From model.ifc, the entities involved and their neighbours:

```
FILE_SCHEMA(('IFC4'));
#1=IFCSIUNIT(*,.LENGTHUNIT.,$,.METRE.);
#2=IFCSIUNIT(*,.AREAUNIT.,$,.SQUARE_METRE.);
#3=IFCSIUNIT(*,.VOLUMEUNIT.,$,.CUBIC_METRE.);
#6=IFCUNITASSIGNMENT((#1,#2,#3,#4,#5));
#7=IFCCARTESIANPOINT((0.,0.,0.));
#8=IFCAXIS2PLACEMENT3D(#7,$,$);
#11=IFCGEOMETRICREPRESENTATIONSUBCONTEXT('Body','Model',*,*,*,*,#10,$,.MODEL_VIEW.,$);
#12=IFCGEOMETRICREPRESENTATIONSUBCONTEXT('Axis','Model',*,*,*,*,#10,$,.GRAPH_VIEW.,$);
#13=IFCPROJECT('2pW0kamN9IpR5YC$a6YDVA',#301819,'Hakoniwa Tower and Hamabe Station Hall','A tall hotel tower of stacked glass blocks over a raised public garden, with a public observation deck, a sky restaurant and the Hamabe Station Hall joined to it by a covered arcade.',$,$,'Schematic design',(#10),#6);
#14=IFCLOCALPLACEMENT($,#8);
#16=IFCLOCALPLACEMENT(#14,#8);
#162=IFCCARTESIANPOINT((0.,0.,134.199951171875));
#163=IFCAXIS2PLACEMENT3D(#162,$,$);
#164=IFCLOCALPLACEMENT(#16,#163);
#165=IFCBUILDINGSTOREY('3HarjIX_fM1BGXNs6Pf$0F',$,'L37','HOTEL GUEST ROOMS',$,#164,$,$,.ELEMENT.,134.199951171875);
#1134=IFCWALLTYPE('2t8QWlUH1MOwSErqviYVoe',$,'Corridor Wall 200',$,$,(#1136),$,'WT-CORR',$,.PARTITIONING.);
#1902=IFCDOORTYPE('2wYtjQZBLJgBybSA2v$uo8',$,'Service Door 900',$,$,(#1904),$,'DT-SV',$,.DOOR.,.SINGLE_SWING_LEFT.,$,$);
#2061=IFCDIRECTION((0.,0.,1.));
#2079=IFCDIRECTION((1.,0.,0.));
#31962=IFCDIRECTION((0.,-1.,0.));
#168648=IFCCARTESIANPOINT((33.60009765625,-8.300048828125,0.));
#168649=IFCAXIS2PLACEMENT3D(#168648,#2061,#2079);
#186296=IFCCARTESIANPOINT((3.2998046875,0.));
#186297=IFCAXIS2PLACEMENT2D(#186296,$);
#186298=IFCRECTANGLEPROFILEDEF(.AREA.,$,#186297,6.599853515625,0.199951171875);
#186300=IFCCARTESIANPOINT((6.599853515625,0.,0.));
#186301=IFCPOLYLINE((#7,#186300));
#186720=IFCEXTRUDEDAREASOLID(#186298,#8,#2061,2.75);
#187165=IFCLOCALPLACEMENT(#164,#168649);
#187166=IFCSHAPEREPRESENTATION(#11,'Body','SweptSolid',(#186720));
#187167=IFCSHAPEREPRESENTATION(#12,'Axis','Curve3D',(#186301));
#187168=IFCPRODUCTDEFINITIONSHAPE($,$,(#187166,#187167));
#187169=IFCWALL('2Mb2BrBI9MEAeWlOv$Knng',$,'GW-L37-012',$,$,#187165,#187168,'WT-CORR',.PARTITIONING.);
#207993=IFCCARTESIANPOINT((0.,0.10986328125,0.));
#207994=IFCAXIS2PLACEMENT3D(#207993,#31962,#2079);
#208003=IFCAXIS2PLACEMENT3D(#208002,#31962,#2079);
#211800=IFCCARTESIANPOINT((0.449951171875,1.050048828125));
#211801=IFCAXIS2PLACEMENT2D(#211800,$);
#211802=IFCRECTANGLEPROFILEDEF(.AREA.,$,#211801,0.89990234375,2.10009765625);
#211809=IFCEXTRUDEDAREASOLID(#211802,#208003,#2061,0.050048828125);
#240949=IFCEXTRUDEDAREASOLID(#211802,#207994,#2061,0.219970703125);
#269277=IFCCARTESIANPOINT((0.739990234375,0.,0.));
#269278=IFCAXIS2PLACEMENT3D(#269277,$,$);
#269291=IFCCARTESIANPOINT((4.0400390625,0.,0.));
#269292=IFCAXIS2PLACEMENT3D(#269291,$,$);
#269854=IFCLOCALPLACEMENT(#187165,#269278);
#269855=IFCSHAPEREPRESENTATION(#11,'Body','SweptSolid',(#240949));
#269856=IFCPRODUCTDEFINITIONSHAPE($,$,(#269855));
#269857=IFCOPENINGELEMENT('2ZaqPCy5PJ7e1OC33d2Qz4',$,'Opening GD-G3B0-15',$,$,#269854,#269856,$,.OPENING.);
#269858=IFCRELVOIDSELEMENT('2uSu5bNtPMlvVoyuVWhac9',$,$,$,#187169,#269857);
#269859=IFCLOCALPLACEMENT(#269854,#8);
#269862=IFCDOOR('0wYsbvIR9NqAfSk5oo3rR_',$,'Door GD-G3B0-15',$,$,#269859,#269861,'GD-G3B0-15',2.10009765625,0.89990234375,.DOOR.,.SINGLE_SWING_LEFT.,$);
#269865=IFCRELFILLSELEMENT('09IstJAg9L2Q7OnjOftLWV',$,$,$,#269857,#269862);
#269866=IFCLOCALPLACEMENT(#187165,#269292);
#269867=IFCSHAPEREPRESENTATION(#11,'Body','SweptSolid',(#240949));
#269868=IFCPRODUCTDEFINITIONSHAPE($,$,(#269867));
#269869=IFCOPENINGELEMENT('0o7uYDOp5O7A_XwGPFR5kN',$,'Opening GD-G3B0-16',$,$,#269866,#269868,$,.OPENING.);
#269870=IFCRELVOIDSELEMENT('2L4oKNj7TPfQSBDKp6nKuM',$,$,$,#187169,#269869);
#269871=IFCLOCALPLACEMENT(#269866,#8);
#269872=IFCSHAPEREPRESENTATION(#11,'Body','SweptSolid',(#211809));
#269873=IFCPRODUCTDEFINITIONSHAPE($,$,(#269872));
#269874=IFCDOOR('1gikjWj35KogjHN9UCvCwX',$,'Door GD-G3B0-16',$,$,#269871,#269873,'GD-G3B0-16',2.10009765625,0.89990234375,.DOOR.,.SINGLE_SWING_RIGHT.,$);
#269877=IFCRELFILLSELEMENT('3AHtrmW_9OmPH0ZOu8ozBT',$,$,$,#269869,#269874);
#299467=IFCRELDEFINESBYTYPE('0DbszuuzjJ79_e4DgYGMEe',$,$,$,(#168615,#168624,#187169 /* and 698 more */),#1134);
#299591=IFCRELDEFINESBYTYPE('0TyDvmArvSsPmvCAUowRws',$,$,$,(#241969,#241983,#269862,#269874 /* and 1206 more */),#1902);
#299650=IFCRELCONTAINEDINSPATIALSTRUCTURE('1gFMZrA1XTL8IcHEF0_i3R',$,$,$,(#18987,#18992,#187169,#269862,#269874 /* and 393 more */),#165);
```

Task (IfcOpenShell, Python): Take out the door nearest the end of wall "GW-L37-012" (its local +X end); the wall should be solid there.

```python
import ifcopenshell
import ifcopenshell.api.feature
import ifcopenshell.api.root
import ifcopenshell.geom
import ifcopenshell.util.shape

model = ifcopenshell.open("model.ifc")
settings = ifcopenshell.geom.settings()


def volume(element):
    """Net volume in cubic metres, openings subtracted."""
    shape = ifcopenshell.geom.create_shape(settings, element)
    return ifcopenshell.util.shape.get_volume(shape.geometry)


door = model.by_guid("1gikjWj35KogjHN9UCvCwX")
opening = door.FillsVoids[0].RelatingOpeningElement
wall = opening.VoidsElements[0].RelatingBuildingElement
before = volume(wall)

ifcopenshell.api.root.remove_product(model, product=door)
ifcopenshell.api.feature.remove_feature(model, feature=opening)

after = volume(wall)

print(f"wall volume {before:.3f} -> {after:.3f} m3")

model.write("model_rev.ifc")
```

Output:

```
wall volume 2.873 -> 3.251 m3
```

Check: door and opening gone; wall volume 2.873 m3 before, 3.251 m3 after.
